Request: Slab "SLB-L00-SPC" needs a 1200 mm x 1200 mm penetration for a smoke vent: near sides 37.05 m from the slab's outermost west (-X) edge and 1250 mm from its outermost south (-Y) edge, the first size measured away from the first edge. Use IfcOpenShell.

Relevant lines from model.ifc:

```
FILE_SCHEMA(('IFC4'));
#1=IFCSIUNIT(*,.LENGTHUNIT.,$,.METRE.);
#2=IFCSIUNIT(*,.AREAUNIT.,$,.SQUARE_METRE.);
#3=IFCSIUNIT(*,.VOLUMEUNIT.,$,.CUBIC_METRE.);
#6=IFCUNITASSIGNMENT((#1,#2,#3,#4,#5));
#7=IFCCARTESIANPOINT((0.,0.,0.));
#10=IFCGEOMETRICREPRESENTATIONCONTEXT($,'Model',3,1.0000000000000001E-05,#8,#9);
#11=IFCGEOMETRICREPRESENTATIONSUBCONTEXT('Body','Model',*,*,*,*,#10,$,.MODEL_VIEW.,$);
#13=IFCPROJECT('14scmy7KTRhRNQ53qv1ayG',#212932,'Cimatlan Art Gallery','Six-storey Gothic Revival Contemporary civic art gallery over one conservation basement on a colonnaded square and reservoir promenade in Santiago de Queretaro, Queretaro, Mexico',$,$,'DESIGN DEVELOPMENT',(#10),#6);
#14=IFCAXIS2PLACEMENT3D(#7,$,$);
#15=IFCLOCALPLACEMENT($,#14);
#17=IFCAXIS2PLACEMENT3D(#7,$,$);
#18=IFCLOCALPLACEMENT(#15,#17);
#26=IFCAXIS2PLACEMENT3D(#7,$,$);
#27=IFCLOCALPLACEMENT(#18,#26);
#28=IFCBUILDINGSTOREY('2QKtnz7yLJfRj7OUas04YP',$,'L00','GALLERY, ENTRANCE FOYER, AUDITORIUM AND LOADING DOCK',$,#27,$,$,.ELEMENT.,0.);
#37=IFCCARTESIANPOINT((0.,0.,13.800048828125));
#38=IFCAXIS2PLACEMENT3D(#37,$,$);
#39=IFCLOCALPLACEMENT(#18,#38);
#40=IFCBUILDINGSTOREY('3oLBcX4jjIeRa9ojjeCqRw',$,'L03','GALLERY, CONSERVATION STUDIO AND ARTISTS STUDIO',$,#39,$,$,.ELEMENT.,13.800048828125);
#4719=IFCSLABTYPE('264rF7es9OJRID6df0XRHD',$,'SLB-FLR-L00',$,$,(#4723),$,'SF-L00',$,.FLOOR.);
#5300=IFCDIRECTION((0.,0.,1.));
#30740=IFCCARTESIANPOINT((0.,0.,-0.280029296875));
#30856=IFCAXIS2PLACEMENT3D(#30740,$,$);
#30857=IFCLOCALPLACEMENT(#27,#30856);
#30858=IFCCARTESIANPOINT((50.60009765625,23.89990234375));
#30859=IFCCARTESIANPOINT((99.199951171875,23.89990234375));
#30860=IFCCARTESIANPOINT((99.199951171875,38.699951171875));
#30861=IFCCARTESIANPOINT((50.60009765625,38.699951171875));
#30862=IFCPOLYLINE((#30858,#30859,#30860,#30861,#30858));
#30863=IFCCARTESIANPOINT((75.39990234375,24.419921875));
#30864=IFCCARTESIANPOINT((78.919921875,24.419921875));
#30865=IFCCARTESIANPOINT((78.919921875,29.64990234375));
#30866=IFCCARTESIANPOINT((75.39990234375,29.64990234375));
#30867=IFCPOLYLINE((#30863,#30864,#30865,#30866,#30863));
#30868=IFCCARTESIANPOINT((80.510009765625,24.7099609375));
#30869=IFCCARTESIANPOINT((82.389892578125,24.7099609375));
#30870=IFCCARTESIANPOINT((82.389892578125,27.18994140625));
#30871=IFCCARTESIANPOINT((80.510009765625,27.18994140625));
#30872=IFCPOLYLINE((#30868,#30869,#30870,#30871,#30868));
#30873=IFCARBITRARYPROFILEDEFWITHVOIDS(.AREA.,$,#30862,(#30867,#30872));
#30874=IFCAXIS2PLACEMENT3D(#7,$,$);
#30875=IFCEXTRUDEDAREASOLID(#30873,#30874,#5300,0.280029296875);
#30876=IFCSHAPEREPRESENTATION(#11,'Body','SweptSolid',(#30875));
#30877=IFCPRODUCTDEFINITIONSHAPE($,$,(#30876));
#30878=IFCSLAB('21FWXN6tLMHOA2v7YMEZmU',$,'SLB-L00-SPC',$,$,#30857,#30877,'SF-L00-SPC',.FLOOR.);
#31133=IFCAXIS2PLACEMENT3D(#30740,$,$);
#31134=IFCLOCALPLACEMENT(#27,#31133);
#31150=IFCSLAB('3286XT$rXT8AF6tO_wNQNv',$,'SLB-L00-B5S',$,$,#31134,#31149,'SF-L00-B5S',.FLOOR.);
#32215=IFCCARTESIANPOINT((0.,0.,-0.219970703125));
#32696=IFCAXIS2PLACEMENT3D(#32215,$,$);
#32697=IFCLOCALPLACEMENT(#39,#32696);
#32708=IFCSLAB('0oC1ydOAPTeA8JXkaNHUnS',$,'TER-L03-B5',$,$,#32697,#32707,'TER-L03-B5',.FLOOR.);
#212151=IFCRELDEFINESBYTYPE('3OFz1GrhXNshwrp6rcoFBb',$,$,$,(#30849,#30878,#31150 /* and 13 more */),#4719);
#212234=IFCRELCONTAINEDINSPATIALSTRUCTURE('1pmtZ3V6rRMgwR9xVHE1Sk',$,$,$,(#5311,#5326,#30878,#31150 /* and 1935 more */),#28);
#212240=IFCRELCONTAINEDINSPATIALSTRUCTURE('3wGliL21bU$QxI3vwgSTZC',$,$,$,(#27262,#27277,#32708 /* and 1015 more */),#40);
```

```python
import numpy as np
import ifcopenshell
import ifcopenshell.api.feature
import ifcopenshell.api.geometry
import ifcopenshell.api.root
import ifcopenshell.geom
import ifcopenshell.util.placement
import ifcopenshell.util.representation
import ifcopenshell.util.shape
import ifcopenshell.util.unit

model = ifcopenshell.open("model.ifc")
unit_scale = ifcopenshell.util.unit.calculate_unit_scale(model)
settings = ifcopenshell.geom.settings()


def volume(element):
    """Net volume in cubic metres, openings subtracted."""
    shape = ifcopenshell.geom.create_shape(settings, element)
    return ifcopenshell.util.shape.get_volume(shape.geometry)


slab = model.by_id(30878)
before = volume(slab)

# Extent in the slab's own axes, in metres. The edges named are its -X and -Y sides.
slab_shape = ifcopenshell.geom.create_shape(settings, slab)
vertices = ifcopenshell.util.shape.get_vertices(slab_shape.geometry)
x_min, y_min, bottom = vertices.min(axis=0)
top = vertices[:, 2].max()

opening = ifcopenshell.api.root.create_entity(model, ifc_class="IfcOpeningElement", name="Smoke vent opening", predefined_type="OPENING")
context = ifcopenshell.util.representation.get_context(model, "Model", "Body", "MODEL_VIEW")
width, depth = 1.2, 1.2
outline = [(0.0, 0.0), (width, 0.0), (width, depth), (0.0, depth), (0.0, 0.0)]
# Overshoot both faces by 50 mm so the cut is clean.
shape = ifcopenshell.api.geometry.add_slab_representation(
    model, context=context, depth=top - bottom + 0.1, polyline=outline
)
ifcopenshell.api.geometry.assign_representation(model, product=opening, representation=shape)

matrix = ifcopenshell.util.placement.get_local_placement(slab.ObjectPlacement)
matrix[:, 3] = matrix @ np.append(np.array([x_min + 37.05, y_min + 1.25, bottom - 0.05]) / unit_scale, 1.0)
ifcopenshell.api.geometry.edit_object_placement(model, product=opening, matrix=matrix, is_si=False)
ifcopenshell.api.feature.add_feature(model, feature=opening, element=slab)

after = volume(slab)

print(f"slab volume {before:.3f} -> {after:.3f} m3")

model.write("model_updated.ifc")
```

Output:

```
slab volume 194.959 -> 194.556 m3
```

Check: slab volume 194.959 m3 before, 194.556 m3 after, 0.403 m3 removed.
